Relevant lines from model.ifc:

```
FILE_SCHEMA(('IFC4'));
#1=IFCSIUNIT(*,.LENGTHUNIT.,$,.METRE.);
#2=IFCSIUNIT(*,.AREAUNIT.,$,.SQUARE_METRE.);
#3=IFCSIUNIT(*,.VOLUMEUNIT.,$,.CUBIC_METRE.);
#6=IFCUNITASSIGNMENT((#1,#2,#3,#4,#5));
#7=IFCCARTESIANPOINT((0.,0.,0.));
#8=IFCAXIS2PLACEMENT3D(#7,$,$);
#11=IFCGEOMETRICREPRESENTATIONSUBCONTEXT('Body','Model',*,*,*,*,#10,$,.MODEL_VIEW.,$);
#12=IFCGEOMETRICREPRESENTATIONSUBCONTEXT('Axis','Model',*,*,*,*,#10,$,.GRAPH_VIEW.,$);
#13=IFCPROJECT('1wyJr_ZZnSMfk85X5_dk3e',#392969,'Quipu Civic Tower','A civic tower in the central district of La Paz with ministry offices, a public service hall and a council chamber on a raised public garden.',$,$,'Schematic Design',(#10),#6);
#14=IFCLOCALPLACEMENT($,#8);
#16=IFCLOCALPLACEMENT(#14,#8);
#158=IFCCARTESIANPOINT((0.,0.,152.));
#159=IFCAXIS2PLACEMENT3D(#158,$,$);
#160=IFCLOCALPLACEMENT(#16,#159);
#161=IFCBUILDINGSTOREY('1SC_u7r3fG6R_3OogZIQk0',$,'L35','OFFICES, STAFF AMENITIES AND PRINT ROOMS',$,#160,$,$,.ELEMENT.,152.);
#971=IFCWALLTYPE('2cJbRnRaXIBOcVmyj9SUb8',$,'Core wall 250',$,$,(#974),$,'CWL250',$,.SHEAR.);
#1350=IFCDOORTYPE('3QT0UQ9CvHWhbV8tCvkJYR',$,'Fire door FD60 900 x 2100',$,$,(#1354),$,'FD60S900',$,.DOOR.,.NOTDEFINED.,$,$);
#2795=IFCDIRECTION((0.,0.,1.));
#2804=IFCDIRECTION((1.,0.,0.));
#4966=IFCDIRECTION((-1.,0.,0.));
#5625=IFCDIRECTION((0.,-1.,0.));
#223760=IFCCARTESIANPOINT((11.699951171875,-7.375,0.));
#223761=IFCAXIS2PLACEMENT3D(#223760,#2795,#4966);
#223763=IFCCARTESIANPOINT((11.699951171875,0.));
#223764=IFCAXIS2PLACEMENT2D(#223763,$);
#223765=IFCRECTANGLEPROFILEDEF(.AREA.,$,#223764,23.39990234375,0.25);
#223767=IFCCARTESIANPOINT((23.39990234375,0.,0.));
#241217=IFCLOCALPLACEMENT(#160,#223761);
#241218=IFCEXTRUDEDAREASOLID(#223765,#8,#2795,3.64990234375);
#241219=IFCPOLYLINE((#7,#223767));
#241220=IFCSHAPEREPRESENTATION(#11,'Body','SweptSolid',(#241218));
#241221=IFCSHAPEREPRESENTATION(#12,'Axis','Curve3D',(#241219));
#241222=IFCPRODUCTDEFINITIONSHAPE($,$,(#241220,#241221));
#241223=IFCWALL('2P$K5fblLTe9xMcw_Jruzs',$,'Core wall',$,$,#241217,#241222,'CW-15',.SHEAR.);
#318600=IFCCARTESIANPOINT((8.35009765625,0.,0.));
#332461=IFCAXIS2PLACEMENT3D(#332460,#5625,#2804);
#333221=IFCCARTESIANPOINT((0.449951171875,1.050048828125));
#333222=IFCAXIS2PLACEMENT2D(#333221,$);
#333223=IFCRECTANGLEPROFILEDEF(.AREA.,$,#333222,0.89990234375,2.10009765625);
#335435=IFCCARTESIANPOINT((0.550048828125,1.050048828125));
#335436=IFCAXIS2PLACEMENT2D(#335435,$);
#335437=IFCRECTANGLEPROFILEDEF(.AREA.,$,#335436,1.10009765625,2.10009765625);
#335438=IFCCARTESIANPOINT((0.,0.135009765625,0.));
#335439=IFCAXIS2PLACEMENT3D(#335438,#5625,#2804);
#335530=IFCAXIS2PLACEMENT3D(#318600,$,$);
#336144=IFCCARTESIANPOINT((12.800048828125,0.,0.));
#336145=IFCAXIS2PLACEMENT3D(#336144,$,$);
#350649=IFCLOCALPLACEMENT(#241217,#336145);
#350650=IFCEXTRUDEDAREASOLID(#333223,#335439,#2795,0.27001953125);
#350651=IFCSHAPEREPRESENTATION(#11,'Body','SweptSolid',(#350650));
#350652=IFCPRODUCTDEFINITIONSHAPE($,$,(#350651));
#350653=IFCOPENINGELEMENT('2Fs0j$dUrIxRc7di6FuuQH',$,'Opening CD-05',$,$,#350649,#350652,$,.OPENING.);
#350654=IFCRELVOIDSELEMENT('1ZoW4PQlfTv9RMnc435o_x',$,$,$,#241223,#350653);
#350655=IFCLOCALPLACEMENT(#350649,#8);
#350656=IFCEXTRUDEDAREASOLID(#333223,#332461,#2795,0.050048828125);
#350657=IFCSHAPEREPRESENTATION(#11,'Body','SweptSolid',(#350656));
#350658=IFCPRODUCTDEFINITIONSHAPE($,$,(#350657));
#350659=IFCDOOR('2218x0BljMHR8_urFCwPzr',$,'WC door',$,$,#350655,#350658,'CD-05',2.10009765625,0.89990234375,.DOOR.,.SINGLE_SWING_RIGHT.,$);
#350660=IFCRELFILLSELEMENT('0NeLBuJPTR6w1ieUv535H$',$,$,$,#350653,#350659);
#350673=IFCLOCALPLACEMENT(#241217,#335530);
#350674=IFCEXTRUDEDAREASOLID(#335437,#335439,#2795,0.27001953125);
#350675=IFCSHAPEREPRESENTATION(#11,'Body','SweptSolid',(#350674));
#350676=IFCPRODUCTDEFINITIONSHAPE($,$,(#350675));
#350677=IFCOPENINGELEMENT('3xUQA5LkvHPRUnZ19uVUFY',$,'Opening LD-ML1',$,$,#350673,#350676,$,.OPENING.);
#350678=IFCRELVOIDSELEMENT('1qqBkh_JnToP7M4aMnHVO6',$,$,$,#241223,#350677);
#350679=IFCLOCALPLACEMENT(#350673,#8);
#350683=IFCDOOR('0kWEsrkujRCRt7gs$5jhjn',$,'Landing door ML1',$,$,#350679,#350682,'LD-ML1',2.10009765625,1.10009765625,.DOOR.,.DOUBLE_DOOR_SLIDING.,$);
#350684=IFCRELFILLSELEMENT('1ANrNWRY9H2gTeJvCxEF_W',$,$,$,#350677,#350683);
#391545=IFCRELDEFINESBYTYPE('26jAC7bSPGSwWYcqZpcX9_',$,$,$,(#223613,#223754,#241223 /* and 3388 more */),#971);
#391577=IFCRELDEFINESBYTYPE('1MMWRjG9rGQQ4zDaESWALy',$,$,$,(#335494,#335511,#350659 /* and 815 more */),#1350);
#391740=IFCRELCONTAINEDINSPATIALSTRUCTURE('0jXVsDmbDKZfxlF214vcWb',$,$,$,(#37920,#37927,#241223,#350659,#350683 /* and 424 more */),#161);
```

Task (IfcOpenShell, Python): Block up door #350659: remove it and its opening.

```python
import ifcopenshell
import ifcopenshell.api.feature
import ifcopenshell.api.root
import ifcopenshell.geom
import ifcopenshell.util.shape

model = ifcopenshell.open("model.ifc")
settings = ifcopenshell.geom.settings()


def volume(element):
    """Net volume in cubic metres, openings subtracted."""
    shape = ifcopenshell.geom.create_shape(settings, element)
    return ifcopenshell.util.shape.get_volume(shape.geometry)


door = model.by_guid("2218x0BljMHR8_urFCwPzr")
opening = door.FillsVoids[0].RelatingOpeningElement
wall = opening.VoidsElements[0].RelatingBuildingElement
before = volume(wall)

ifcopenshell.api.root.remove_product(model, product=door)
ifcopenshell.api.feature.remove_feature(model, feature=opening)

after = volume(wall)

print(f"wall volume {before:.3f} -> {after:.3f} m3")

model.write("model_v2.ifc")
```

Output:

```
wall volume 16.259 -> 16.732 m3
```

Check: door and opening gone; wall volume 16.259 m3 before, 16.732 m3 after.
